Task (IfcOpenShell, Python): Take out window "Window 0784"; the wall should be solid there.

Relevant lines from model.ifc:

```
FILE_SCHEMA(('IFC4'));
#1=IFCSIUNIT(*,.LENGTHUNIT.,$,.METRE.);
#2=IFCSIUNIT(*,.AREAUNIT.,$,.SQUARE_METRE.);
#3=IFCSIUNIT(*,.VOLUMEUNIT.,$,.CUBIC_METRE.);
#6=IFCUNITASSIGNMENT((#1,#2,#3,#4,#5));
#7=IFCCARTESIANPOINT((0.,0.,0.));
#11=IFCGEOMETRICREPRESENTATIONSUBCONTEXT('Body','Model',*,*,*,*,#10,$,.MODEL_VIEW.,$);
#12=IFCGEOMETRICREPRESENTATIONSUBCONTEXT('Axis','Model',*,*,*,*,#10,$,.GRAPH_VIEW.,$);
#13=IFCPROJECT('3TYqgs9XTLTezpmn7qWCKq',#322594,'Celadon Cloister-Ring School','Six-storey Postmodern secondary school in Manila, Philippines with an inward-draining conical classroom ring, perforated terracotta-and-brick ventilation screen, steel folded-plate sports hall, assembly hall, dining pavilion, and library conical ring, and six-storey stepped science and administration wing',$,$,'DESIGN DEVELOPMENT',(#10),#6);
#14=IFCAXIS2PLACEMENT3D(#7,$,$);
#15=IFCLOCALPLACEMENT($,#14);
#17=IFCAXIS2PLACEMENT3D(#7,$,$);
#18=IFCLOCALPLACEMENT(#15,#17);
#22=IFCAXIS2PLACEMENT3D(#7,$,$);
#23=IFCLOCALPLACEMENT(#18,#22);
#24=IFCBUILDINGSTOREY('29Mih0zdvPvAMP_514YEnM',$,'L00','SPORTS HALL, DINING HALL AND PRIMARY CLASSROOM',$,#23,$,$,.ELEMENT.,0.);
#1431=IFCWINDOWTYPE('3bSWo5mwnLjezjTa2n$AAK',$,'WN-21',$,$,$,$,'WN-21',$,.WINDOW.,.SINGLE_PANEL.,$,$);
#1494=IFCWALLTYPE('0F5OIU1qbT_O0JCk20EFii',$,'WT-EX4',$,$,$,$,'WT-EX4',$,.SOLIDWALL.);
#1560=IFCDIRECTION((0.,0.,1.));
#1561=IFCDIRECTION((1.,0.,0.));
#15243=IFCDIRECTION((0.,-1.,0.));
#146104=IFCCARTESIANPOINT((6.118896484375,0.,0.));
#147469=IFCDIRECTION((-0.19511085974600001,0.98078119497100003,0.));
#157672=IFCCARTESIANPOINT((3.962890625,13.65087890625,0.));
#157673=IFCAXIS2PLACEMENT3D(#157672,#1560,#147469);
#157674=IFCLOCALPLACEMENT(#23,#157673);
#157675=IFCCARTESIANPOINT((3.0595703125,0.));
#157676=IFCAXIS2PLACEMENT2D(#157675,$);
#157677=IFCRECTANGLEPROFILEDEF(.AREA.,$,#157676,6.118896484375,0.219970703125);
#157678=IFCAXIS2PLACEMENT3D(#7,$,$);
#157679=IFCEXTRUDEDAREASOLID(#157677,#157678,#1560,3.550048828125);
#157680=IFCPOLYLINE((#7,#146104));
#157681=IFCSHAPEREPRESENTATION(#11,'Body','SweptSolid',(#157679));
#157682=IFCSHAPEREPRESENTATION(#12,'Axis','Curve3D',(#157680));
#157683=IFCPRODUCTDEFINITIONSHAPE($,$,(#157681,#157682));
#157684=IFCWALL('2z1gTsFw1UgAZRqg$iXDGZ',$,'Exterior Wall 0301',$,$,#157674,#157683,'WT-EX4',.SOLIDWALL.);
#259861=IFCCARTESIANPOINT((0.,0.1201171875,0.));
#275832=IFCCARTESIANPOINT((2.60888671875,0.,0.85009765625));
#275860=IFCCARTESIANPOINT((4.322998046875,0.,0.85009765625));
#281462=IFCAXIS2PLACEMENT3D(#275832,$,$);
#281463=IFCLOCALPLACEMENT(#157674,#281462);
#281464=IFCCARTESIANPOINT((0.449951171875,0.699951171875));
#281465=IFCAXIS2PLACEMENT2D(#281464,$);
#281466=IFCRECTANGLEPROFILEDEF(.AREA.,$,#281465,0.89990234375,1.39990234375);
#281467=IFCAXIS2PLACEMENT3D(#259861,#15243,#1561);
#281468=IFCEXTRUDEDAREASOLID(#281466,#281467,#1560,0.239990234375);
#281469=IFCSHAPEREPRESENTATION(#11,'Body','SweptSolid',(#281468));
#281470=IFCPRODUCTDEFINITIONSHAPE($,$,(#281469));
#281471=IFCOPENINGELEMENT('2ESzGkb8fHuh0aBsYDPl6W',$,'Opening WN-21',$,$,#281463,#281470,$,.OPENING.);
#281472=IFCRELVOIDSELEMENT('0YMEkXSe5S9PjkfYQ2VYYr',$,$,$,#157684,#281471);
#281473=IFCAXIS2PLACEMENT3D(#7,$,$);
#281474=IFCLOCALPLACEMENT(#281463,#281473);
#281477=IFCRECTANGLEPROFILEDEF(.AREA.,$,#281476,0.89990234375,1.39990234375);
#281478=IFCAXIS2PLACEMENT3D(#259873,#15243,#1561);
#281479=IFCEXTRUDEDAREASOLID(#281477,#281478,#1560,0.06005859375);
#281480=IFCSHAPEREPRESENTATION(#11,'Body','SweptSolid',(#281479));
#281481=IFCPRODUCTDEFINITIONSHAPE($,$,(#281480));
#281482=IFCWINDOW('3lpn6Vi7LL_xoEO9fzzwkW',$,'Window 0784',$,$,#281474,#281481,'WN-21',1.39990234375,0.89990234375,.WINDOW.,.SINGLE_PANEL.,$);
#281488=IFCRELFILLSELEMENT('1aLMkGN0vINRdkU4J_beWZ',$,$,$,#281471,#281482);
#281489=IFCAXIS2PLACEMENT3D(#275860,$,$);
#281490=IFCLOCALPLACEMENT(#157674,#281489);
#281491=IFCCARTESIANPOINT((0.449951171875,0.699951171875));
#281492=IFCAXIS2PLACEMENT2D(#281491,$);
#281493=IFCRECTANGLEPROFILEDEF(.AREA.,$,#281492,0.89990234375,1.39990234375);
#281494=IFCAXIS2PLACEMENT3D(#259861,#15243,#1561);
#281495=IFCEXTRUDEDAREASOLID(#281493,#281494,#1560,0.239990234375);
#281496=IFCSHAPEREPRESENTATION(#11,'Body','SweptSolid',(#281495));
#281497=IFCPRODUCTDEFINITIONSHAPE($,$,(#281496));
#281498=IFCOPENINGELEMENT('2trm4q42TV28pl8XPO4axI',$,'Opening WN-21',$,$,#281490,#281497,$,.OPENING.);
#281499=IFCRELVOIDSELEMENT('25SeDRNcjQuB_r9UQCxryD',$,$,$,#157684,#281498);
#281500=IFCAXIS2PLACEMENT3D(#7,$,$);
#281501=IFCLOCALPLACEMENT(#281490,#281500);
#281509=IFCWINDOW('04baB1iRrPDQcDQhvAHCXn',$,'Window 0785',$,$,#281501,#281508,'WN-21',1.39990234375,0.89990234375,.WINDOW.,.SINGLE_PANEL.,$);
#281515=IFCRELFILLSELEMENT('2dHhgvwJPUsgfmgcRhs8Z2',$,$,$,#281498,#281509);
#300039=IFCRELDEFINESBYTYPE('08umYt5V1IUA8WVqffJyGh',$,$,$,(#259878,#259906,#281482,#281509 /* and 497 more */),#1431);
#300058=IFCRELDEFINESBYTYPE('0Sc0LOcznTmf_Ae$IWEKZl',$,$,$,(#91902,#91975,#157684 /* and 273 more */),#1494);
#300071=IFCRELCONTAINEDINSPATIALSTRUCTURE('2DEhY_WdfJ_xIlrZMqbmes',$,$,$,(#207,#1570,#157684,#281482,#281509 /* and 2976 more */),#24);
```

```python
import ifcopenshell
import ifcopenshell.api.feature
import ifcopenshell.api.root
import ifcopenshell.geom
import ifcopenshell.util.shape

model = ifcopenshell.open("model.ifc")
settings = ifcopenshell.geom.settings()


def volume(element):
    """Net volume in cubic metres, openings subtracted."""
    shape = ifcopenshell.geom.create_shape(settings, element)
    return ifcopenshell.util.shape.get_volume(shape.geometry)


window = model.by_id(281482)
opening = window.FillsVoids[0].RelatingOpeningElement
wall = opening.VoidsElements[0].RelatingBuildingElement
before = volume(wall)

ifcopenshell.api.root.remove_product(model, product=window)
ifcopenshell.api.feature.remove_feature(model, feature=opening)

after = volume(wall)

print(f"wall volume {before:.3f} -> {after:.3f} m3")

model.write("model_v2.ifc")
```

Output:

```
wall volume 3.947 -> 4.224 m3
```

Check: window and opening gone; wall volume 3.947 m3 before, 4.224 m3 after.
